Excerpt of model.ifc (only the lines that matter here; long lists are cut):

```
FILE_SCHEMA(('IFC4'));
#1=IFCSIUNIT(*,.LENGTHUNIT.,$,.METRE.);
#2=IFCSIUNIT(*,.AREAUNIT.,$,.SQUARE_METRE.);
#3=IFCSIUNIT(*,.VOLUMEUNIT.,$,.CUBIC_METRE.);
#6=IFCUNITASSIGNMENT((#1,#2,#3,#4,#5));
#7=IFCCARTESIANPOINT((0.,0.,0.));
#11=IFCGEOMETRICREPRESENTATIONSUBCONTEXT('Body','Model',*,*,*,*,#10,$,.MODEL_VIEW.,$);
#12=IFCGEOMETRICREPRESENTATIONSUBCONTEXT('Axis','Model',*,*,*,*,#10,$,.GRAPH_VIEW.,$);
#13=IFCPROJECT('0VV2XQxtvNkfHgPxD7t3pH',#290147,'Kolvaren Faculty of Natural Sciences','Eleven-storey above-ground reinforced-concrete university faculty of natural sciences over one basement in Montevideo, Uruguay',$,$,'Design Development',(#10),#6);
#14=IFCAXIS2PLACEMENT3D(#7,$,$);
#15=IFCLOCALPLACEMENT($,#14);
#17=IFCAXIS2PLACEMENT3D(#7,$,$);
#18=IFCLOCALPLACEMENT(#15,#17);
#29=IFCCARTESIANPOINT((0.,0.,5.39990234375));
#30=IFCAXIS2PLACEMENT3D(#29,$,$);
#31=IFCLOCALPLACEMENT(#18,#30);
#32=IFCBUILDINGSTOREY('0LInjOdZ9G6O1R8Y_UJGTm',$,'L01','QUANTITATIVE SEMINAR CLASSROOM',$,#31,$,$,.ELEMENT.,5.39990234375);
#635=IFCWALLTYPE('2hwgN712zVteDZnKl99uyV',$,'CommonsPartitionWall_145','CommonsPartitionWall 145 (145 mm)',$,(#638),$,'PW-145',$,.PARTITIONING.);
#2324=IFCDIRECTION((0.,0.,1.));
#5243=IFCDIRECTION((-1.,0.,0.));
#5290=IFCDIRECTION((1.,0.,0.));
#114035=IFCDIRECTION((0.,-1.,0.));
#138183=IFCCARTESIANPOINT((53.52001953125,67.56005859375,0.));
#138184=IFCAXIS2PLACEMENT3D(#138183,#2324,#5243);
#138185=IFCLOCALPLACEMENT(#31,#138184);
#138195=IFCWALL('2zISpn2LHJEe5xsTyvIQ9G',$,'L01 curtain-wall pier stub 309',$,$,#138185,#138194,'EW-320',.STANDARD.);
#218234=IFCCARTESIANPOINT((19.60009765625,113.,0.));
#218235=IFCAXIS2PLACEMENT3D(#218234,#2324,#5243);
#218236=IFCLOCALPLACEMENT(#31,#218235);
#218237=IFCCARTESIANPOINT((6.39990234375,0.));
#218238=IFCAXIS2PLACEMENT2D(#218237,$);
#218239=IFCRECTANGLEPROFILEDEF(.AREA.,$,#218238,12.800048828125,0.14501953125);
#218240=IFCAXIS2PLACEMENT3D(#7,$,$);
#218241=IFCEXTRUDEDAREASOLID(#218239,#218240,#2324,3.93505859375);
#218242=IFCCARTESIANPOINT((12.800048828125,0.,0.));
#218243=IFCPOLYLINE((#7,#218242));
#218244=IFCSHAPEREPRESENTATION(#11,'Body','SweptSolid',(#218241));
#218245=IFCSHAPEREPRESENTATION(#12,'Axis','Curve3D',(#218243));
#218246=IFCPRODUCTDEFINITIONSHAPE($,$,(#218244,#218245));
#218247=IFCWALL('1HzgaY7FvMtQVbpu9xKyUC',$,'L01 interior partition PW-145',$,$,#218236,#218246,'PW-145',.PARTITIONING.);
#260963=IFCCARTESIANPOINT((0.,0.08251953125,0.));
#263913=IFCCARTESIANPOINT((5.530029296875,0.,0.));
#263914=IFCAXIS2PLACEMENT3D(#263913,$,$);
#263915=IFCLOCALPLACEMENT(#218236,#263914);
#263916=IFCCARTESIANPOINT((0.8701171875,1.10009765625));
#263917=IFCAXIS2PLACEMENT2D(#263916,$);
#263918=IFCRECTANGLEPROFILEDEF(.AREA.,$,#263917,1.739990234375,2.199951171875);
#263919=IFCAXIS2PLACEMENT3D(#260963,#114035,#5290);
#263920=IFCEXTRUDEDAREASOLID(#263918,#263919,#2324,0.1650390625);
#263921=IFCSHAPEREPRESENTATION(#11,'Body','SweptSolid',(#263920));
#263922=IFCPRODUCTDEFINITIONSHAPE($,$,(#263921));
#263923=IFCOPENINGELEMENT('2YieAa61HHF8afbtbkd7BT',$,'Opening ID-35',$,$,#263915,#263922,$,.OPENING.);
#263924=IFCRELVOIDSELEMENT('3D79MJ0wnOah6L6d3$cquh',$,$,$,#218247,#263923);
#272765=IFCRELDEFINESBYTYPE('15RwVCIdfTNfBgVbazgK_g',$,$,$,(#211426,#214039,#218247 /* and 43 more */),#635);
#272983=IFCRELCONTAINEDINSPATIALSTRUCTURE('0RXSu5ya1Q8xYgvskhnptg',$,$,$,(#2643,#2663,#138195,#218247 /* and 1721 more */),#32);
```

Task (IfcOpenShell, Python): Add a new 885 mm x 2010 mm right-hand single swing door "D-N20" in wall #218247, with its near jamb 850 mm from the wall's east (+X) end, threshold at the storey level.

```python
import numpy as np
import ifcopenshell
import ifcopenshell.api.feature
import ifcopenshell.api.geometry
import ifcopenshell.api.root
import ifcopenshell.api.spatial
import ifcopenshell.geom
import ifcopenshell.util.element
import ifcopenshell.util.placement
import ifcopenshell.util.representation
import ifcopenshell.util.shape
import ifcopenshell.util.unit

model = ifcopenshell.open("model.ifc")
unit_scale = ifcopenshell.util.unit.calculate_unit_scale(model)
settings = ifcopenshell.geom.settings()


def volume(element):
    """Net volume in cubic metres, openings subtracted."""
    shape = ifcopenshell.geom.create_shape(settings, element)
    return ifcopenshell.util.shape.get_volume(shape.geometry)


wall = model.by_guid("1HzgaY7FvMtQVbpu9xKyUC")
storey = ifcopenshell.util.element.get_container(wall, ifc_class="IfcBuildingStorey")
context = ifcopenshell.util.representation.get_context(model, "Model", "Body", "MODEL_VIEW")
before = volume(wall)

width, height, from_end, sill = 0.885, 2.01, 0.85, 0.0  # metres

# The wall runs along its own X axis, and the end named is its -X end.
wall_shape = ifcopenshell.geom.create_shape(settings, wall)
x, y, z = ifcopenshell.util.shape.get_vertices(wall_shape.geometry).T
start = x.min() + from_end
face, thickness = float(y.min()), float(y.max() - y.min())
wall_matrix = ifcopenshell.util.placement.get_local_placement(wall.ObjectPlacement)
level = ifcopenshell.util.placement.get_local_placement(storey.ObjectPlacement)[2, 3]


def in_wall(x, y):
    """Placement at x, y metres in the wall's axes, at sill height."""
    matrix = wall_matrix.copy()
    matrix[:, 3] = wall_matrix @ np.array([x / unit_scale, y / unit_scale, 0.0, 1.0])
    matrix[2, 3] = level + sill / unit_scale
    return matrix


# Opening: a box that overshoots both wall faces by 50 mm.
opening = ifcopenshell.api.root.create_entity(model, ifc_class="IfcOpeningElement", predefined_type="OPENING")
box = ifcopenshell.api.geometry.add_wall_representation(
    model, context=context, length=width, height=height, thickness=thickness + 0.1
)
ifcopenshell.api.geometry.assign_representation(model, product=opening, representation=box)
ifcopenshell.api.geometry.edit_object_placement(model, product=opening, matrix=in_wall(start, face - 0.05), is_si=False)
ifcopenshell.api.feature.add_feature(model, feature=opening, element=wall)

door = ifcopenshell.api.root.create_entity(model, ifc_class="IfcDoor", name="D-N20", predefined_type="DOOR")
door.OverallWidth, door.OverallHeight = width / unit_scale, height / unit_scale
door.OperationType = "SINGLE_SWING_RIGHT"
body = ifcopenshell.api.geometry.add_door_representation(
    model,
    context=context,
    overall_width=door.OverallWidth,
    overall_height=door.OverallHeight,
    operation_type="SINGLE_SWING_RIGHT",
    lining_properties={"LiningDepth": thickness / unit_scale, "ThresholdDepth": thickness / unit_scale},
)
ifcopenshell.api.geometry.assign_representation(model, product=door, representation=body)
ifcopenshell.api.spatial.assign_container(model, products=[door], relating_structure=storey)
ifcopenshell.api.feature.add_filling(model, opening=opening, element=door)

# The lining spans the wall, so the door starts at the wall face.
ifcopenshell.api.geometry.edit_object_placement(model, product=door, matrix=in_wall(start, face), is_si=False)

after = volume(wall)

print(f"wall volume {before:.3f} -> {after:.3f} m3")

model.write("model_edited.ifc")
```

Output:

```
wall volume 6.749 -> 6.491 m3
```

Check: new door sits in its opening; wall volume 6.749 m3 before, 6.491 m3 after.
